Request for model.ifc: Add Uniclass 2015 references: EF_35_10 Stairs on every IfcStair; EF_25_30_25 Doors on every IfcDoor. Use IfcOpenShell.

First a look at what the model holds.

```python
import ifcopenshell

model = ifcopenshell.open("model.ifc")
print(model.schema)
print("classifications:", [c.Name for c in model.by_type("IfcClassification")])
for ifc_class in ("IfcDoor", "IfcRoof", "IfcStair", "IfcWall", "IfcWindow"):
    print(ifc_class, len(model.by_type(ifc_class)))
```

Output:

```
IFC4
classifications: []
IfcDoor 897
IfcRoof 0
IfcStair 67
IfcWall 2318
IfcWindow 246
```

```python
import ifcopenshell
import ifcopenshell.api.classification

model = ifcopenshell.open("model.ifc")

system = ifcopenshell.api.classification.add_classification(model, classification="Uniclass 2015")

codes = {
    "IfcStair": ("EF_35_10", "Stairs"),
    "IfcDoor": ("EF_25_30_25", "Doors"),
}
for ifc_class, (code, name) in codes.items():
    products = model.by_type(ifc_class)
    ifcopenshell.api.classification.add_reference(
        model, products=products, classification=system, identification=code, name=name
    )
    print(code, len(products))

model.write("model_rev.ifc")
```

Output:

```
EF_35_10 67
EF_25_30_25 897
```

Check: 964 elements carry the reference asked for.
